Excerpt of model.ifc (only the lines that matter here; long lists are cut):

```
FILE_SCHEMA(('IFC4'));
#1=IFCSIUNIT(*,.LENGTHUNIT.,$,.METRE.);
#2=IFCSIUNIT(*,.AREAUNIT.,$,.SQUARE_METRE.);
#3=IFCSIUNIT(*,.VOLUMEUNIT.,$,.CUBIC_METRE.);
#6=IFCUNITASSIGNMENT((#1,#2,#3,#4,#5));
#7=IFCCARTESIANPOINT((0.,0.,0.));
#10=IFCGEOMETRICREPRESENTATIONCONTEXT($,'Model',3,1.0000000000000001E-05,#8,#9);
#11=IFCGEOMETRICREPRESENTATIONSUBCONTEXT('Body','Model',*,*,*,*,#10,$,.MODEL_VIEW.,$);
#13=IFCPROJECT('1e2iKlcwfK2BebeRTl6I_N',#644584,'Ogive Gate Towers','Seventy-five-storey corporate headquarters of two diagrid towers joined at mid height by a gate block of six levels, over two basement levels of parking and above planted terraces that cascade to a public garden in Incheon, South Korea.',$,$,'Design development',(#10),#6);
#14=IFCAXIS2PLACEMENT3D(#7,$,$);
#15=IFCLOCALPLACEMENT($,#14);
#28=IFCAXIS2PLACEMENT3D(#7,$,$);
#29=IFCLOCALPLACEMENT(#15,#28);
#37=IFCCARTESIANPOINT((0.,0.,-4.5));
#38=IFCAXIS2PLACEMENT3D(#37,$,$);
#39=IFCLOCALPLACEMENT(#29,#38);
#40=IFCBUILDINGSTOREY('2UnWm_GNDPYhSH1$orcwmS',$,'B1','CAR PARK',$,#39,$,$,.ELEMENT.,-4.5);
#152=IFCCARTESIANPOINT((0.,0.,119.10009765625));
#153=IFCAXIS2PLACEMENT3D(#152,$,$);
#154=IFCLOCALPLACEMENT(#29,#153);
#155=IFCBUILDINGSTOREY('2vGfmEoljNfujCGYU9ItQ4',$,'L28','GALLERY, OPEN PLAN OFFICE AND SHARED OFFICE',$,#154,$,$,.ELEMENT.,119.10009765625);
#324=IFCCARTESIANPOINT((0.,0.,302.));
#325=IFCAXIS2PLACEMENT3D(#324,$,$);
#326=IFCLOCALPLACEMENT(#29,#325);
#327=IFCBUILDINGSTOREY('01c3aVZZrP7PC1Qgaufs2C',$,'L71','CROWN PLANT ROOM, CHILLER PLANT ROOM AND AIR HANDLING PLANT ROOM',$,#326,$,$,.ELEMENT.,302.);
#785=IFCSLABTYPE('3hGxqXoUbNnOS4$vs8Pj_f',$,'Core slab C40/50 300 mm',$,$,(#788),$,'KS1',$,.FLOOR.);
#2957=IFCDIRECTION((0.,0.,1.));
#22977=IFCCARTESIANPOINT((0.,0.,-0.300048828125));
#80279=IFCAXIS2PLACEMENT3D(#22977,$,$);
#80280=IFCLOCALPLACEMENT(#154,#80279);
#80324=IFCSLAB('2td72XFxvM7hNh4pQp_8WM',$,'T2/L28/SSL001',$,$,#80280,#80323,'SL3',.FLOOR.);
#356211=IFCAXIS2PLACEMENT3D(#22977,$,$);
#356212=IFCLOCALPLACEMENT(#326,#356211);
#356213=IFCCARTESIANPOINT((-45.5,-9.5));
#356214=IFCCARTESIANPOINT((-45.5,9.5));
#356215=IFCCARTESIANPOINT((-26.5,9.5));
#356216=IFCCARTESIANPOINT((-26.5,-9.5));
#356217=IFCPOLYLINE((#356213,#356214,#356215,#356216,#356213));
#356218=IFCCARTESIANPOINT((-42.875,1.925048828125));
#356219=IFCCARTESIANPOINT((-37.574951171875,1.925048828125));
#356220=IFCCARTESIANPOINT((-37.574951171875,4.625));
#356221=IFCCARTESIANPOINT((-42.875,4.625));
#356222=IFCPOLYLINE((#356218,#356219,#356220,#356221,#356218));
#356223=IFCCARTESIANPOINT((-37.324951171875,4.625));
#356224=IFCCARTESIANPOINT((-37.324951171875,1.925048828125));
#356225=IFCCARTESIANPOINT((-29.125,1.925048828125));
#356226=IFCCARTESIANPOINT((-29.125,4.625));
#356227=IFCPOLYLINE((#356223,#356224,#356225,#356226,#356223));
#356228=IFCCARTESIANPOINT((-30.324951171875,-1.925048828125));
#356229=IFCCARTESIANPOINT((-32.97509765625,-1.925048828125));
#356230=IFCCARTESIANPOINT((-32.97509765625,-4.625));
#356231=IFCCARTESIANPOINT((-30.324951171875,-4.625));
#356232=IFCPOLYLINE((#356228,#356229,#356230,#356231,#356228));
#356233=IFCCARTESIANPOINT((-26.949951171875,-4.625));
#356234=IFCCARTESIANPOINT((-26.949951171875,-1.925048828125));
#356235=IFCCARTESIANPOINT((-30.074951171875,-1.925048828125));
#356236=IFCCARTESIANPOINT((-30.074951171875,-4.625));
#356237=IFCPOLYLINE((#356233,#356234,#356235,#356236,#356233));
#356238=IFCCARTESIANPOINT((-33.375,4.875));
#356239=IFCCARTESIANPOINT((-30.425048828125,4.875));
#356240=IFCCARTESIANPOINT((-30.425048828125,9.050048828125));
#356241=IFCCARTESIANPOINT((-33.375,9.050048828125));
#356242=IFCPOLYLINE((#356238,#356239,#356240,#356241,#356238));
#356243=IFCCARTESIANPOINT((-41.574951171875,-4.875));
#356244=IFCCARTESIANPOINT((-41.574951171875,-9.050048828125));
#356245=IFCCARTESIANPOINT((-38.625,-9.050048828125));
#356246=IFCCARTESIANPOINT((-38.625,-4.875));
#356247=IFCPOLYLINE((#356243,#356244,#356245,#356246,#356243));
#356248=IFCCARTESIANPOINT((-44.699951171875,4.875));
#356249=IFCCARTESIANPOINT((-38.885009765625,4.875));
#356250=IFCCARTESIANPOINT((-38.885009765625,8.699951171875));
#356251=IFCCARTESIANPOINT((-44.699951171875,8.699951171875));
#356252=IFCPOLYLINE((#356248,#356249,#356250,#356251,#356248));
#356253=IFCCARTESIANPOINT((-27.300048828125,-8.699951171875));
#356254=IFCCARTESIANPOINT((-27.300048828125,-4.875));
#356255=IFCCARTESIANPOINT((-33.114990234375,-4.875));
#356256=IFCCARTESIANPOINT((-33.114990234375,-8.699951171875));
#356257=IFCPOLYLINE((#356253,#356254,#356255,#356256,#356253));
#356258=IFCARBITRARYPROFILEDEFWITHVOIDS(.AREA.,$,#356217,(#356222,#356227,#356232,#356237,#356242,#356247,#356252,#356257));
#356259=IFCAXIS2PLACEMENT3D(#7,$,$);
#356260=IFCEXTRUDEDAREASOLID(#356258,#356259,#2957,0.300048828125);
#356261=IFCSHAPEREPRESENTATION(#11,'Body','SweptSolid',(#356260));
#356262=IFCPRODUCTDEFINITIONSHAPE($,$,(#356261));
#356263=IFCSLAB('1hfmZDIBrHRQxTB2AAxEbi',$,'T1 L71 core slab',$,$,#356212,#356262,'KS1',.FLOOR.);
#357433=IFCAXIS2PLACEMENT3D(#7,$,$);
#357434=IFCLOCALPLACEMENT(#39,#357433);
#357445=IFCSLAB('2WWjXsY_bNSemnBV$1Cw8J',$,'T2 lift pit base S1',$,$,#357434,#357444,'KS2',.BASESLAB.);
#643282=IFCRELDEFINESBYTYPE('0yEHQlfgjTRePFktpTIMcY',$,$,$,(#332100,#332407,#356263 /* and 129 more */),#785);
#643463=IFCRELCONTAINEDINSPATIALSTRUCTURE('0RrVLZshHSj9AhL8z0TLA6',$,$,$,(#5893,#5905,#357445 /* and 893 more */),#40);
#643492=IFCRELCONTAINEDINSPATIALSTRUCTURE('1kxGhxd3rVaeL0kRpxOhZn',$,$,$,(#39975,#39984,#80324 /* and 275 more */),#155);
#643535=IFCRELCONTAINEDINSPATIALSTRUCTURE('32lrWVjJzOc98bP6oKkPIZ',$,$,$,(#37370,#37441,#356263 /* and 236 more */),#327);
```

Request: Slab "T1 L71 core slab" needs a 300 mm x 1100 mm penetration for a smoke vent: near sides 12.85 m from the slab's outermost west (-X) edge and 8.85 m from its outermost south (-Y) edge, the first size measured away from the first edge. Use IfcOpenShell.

```python
import numpy as np
import ifcopenshell
import ifcopenshell.api.feature
import ifcopenshell.api.geometry
import ifcopenshell.api.root
import ifcopenshell.geom
import ifcopenshell.util.placement
import ifcopenshell.util.representation
import ifcopenshell.util.shape
import ifcopenshell.util.unit

model = ifcopenshell.open("model.ifc")
unit_scale = ifcopenshell.util.unit.calculate_unit_scale(model)
settings = ifcopenshell.geom.settings()


def volume(element):
    """Net volume in cubic metres, openings subtracted."""
    shape = ifcopenshell.geom.create_shape(settings, element)
    return ifcopenshell.util.shape.get_volume(shape.geometry)


slab = model.by_guid("1hfmZDIBrHRQxTB2AAxEbi")
before = volume(slab)

# Extent in the slab's own axes, in metres. The edges named are its -X and -Y sides.
slab_shape = ifcopenshell.geom.create_shape(settings, slab)
vertices = ifcopenshell.util.shape.get_vertices(slab_shape.geometry)
x_min, y_min, bottom = vertices.min(axis=0)
top = vertices[:, 2].max()

opening = ifcopenshell.api.root.create_entity(model, ifc_class="IfcOpeningElement", name="Smoke vent opening", predefined_type="OPENING")
context = ifcopenshell.util.representation.get_context(model, "Model", "Body", "MODEL_VIEW")
width, depth = 0.3, 1.1
outline = [(0.0, 0.0), (width, 0.0), (width, depth), (0.0, depth), (0.0, 0.0)]
# Overshoot both faces by 50 mm so the cut is clean.
shape = ifcopenshell.api.geometry.add_slab_representation(
    model, context=context, depth=top - bottom + 0.1, polyline=outline
)
ifcopenshell.api.geometry.assign_representation(model, product=opening, representation=shape)

matrix = ifcopenshell.util.placement.get_local_placement(slab.ObjectPlacement)
matrix[:, 3] = matrix @ np.append(np.array([x_min + 12.85, y_min + 8.85, bottom - 0.05]) / unit_scale, 1.0)
ifcopenshell.api.geometry.edit_object_placement(model, product=opening, matrix=matrix, is_si=False)
ifcopenshell.api.feature.add_feature(model, feature=opening, element=slab)

after = volume(slab)

print(f"slab volume {before:.3f} -> {after:.3f} m3")

model.write("model_rev.ifc")
```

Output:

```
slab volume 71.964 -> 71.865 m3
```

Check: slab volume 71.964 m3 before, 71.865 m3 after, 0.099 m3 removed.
